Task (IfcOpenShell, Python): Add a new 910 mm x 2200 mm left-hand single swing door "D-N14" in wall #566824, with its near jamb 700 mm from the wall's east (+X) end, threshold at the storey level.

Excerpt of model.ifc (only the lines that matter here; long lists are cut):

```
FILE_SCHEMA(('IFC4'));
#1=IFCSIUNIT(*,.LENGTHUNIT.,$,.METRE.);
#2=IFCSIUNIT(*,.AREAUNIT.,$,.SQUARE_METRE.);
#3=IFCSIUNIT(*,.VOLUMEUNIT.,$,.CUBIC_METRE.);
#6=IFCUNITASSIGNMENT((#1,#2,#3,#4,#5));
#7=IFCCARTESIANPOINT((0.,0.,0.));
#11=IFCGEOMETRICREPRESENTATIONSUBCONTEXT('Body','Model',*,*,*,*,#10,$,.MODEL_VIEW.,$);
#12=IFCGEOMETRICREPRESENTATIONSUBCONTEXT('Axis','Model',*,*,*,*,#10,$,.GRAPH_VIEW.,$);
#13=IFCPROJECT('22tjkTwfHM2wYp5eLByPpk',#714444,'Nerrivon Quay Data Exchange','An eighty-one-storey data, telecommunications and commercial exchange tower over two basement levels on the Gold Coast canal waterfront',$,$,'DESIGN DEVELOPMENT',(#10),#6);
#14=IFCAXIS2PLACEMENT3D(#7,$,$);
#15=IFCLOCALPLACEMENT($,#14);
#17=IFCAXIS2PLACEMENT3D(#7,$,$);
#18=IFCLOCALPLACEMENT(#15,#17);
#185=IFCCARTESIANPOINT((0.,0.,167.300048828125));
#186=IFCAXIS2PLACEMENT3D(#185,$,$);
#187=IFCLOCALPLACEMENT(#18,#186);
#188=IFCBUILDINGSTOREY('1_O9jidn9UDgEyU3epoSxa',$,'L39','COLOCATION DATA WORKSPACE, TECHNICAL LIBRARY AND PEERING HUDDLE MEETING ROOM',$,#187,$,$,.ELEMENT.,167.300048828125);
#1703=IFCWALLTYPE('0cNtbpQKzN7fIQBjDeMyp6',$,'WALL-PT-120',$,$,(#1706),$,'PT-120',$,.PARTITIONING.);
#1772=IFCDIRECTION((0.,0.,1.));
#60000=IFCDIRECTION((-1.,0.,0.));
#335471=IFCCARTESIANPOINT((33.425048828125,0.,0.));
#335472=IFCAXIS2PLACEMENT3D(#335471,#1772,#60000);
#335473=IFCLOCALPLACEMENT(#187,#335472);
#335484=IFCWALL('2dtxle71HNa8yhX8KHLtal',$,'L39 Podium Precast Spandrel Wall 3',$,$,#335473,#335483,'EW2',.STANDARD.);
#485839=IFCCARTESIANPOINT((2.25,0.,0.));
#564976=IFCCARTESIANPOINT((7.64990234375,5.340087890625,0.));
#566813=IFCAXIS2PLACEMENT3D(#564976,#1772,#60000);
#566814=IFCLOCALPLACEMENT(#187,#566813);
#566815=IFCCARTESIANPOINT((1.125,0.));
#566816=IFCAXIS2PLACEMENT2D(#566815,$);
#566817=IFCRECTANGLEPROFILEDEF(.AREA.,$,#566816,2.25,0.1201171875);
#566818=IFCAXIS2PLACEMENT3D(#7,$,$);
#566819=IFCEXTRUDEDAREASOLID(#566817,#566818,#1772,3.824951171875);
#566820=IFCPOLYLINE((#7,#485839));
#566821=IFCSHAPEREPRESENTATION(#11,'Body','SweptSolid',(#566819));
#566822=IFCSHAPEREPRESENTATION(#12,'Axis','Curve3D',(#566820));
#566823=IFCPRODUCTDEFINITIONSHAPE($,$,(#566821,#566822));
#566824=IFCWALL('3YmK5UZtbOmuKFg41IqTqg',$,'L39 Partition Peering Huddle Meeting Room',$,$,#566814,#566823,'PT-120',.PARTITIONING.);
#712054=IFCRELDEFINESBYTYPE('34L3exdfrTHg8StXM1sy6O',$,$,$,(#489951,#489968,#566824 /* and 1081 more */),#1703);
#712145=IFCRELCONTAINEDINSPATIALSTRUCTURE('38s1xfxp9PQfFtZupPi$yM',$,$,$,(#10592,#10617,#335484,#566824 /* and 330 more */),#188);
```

```python
import numpy as np
import ifcopenshell
import ifcopenshell.api.feature
import ifcopenshell.api.geometry
import ifcopenshell.api.root
import ifcopenshell.api.spatial
import ifcopenshell.geom
import ifcopenshell.util.element
import ifcopenshell.util.placement
import ifcopenshell.util.representation
import ifcopenshell.util.shape
import ifcopenshell.util.unit

model = ifcopenshell.open("model.ifc")
unit_scale = ifcopenshell.util.unit.calculate_unit_scale(model)
settings = ifcopenshell.geom.settings()


def volume(element):
    """Net volume in cubic metres, openings subtracted."""
    shape = ifcopenshell.geom.create_shape(settings, element)
    return ifcopenshell.util.shape.get_volume(shape.geometry)


wall = model.by_guid("3YmK5UZtbOmuKFg41IqTqg")
storey = ifcopenshell.util.element.get_container(wall, ifc_class="IfcBuildingStorey")
context = ifcopenshell.util.representation.get_context(model, "Model", "Body", "MODEL_VIEW")
before = volume(wall)

width, height, from_end, sill = 0.91, 2.2, 0.7, 0.0  # metres

# The wall runs along its own X axis, and the end named is its -X end.
wall_shape = ifcopenshell.geom.create_shape(settings, wall)
x, y, z = ifcopenshell.util.shape.get_vertices(wall_shape.geometry).T
start = x.min() + from_end
face, thickness = float(y.min()), float(y.max() - y.min())
wall_matrix = ifcopenshell.util.placement.get_local_placement(wall.ObjectPlacement)
level = ifcopenshell.util.placement.get_local_placement(storey.ObjectPlacement)[2, 3]


def in_wall(x, y):
    """Placement at x, y metres in the wall's axes, at sill height."""
    matrix = wall_matrix.copy()
    matrix[:, 3] = wall_matrix @ np.array([x / unit_scale, y / unit_scale, 0.0, 1.0])
    matrix[2, 3] = level + sill / unit_scale
    return matrix


# Opening: a box that overshoots both wall faces by 50 mm.
opening = ifcopenshell.api.root.create_entity(model, ifc_class="IfcOpeningElement", predefined_type="OPENING")
box = ifcopenshell.api.geometry.add_wall_representation(
    model, context=context, length=width, height=height, thickness=thickness + 0.1
)
ifcopenshell.api.geometry.assign_representation(model, product=opening, representation=box)
ifcopenshell.api.geometry.edit_object_placement(model, product=opening, matrix=in_wall(start, face - 0.05), is_si=False)
ifcopenshell.api.feature.add_feature(model, feature=opening, element=wall)

door = ifcopenshell.api.root.create_entity(model, ifc_class="IfcDoor", name="D-N14", predefined_type="DOOR")
door.OverallWidth, door.OverallHeight = width / unit_scale, height / unit_scale
door.OperationType = "SINGLE_SWING_LEFT"
body = ifcopenshell.api.geometry.add_door_representation(
    model,
    context=context,
    overall_width=door.OverallWidth,
    overall_height=door.OverallHeight,
    operation_type="SINGLE_SWING_LEFT",
    lining_properties={"LiningDepth": thickness / unit_scale, "ThresholdDepth": thickness / unit_scale},
)
ifcopenshell.api.geometry.assign_representation(model, product=door, representation=body)
ifcopenshell.api.spatial.assign_container(model, products=[door], relating_structure=storey)
ifcopenshell.api.feature.add_filling(model, opening=opening, element=door)

# The lining spans the wall, so the door starts at the wall face.
ifcopenshell.api.geometry.edit_object_placement(model, product=door, matrix=in_wall(start, face), is_si=False)

after = volume(wall)

print(f"wall volume {before:.3f} -> {after:.3f} m3")

model.write("model_updated.ifc")
```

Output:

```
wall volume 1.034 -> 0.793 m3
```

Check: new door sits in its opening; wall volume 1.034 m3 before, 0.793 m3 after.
